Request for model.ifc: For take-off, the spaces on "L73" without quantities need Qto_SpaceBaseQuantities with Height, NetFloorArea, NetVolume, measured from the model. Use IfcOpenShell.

First a look at what the model holds.

```python
import ifcopenshell
import ifcopenshell.util.element
import ifcopenshell.util.unit

model = ifcopenshell.open("model.ifc")
print(model.schema)
for unit_type in ("LENGTHUNIT", "AREAUNIT", "VOLUMEUNIT"):
    print(unit_type, ifcopenshell.util.unit.calculate_unit_scale(model, unit_type))
storey = next(s for s in model.by_type("IfcBuildingStorey") if s.Name == "L73")
spaces = [e for e in ifcopenshell.util.element.get_decomposition(storey) if e.is_a("IfcSpace")]
for e in sorted(spaces, key=lambda e: e.id()):
    print(e.id(), e.is_a(), e.Name, list(ifcopenshell.util.element.get_psets(e, qtos_only=True)), sep=" | ")
```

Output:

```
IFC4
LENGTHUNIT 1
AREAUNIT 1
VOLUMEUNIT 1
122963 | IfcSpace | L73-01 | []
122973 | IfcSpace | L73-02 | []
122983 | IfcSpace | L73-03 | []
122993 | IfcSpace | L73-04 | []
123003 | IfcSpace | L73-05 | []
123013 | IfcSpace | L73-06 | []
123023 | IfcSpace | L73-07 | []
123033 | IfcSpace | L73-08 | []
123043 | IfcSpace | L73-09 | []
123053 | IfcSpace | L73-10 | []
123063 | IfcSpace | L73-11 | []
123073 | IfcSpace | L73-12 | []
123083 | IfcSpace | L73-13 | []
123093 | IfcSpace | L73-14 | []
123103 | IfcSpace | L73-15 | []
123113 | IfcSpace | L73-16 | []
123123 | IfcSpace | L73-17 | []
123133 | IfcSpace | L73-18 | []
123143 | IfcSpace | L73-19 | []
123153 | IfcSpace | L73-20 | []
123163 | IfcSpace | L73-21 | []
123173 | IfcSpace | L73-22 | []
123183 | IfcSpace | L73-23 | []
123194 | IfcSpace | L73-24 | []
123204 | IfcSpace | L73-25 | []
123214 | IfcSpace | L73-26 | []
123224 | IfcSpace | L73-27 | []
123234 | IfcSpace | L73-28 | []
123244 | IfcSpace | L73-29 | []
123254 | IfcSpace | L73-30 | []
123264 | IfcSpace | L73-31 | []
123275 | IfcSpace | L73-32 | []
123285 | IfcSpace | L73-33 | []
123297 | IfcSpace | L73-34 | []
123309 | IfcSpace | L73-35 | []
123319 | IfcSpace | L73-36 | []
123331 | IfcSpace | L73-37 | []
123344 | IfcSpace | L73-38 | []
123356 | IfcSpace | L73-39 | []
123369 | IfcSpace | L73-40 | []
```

```python
import ifcopenshell
import ifcopenshell.api.pset
import ifcopenshell.geom
import ifcopenshell.util.element
import ifcopenshell.util.shape
import ifcopenshell.util.unit

model = ifcopenshell.open("model.ifc")
unit_scale = ifcopenshell.util.unit.calculate_unit_scale(model)
area_scale = ifcopenshell.util.unit.calculate_unit_scale(model, "AREAUNIT")
volume_scale = ifcopenshell.util.unit.calculate_unit_scale(model, "VOLUMEUNIT")
settings = ifcopenshell.geom.settings()

storey = next(s for s in model.by_type("IfcBuildingStorey") if s.Name == "L73")
spaces = [e for e in ifcopenshell.util.element.get_decomposition(storey) if e.is_a("IfcSpace")]

for e in sorted(spaces, key=lambda e: e.id()):
    if ifcopenshell.util.element.get_psets(e, qtos_only=True, should_inherit=False):
        continue
    # Geometry comes back in metres, in the element's own axes.
    shape = ifcopenshell.geom.create_shape(settings, e)
    values = {
        "Height": ifcopenshell.util.shape.get_z(shape.geometry) / unit_scale,
        "NetFloorArea": ifcopenshell.util.shape.get_footprint_area(shape.geometry) / area_scale,
        "NetVolume": ifcopenshell.util.shape.get_volume(shape.geometry) / volume_scale,
    }
    qto = ifcopenshell.api.pset.add_qto(model, product=e, name="Qto_SpaceBaseQuantities")
    ifcopenshell.api.pset.edit_qto(model, qto=qto, properties=values)
    print(e.id(), {k: round(v, 3) for k, v in values.items()})

model.write("model-out.ifc")
```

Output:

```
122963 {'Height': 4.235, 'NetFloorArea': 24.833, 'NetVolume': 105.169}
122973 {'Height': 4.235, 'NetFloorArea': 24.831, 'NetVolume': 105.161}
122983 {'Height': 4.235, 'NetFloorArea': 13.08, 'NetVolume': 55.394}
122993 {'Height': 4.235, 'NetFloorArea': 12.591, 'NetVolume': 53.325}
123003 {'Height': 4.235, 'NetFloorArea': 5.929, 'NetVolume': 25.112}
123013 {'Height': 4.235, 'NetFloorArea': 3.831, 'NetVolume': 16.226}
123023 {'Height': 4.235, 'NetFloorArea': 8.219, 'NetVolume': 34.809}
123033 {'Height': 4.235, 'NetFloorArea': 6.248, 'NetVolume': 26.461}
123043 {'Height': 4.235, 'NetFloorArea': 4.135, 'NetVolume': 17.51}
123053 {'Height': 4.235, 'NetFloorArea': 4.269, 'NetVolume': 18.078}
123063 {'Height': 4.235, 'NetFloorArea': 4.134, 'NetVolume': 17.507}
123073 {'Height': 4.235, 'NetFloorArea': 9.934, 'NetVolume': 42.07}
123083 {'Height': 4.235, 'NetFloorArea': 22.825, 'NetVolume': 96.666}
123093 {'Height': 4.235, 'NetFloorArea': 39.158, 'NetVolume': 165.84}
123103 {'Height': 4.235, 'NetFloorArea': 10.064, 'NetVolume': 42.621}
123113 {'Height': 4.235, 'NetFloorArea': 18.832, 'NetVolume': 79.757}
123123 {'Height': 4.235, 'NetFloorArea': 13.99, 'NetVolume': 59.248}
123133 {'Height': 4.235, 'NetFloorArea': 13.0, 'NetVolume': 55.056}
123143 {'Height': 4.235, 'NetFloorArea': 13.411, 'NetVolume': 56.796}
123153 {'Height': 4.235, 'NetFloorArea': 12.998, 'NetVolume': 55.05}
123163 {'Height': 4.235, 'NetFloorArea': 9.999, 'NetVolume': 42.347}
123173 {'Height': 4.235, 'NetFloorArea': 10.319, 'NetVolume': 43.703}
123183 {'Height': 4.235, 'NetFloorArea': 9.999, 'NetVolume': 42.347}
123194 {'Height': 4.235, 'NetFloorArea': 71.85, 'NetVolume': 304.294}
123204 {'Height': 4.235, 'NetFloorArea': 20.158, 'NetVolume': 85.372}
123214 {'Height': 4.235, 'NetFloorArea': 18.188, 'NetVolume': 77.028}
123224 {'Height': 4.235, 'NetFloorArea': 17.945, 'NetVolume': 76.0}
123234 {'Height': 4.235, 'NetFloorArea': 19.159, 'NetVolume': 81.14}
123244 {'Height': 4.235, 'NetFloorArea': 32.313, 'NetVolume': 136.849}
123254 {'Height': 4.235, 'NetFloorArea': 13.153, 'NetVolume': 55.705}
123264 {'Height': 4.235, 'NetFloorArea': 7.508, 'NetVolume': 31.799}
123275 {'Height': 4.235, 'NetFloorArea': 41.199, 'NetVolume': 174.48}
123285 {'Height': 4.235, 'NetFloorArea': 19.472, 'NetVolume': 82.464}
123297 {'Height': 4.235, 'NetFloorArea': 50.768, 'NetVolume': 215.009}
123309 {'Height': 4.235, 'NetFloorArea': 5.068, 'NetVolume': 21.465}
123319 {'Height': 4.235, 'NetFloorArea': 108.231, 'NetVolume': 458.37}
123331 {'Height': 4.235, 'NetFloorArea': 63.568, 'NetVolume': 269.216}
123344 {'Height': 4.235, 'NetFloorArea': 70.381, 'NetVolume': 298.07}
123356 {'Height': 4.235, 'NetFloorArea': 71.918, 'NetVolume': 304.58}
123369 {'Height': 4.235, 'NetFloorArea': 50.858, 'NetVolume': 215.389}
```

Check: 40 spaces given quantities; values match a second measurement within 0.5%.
